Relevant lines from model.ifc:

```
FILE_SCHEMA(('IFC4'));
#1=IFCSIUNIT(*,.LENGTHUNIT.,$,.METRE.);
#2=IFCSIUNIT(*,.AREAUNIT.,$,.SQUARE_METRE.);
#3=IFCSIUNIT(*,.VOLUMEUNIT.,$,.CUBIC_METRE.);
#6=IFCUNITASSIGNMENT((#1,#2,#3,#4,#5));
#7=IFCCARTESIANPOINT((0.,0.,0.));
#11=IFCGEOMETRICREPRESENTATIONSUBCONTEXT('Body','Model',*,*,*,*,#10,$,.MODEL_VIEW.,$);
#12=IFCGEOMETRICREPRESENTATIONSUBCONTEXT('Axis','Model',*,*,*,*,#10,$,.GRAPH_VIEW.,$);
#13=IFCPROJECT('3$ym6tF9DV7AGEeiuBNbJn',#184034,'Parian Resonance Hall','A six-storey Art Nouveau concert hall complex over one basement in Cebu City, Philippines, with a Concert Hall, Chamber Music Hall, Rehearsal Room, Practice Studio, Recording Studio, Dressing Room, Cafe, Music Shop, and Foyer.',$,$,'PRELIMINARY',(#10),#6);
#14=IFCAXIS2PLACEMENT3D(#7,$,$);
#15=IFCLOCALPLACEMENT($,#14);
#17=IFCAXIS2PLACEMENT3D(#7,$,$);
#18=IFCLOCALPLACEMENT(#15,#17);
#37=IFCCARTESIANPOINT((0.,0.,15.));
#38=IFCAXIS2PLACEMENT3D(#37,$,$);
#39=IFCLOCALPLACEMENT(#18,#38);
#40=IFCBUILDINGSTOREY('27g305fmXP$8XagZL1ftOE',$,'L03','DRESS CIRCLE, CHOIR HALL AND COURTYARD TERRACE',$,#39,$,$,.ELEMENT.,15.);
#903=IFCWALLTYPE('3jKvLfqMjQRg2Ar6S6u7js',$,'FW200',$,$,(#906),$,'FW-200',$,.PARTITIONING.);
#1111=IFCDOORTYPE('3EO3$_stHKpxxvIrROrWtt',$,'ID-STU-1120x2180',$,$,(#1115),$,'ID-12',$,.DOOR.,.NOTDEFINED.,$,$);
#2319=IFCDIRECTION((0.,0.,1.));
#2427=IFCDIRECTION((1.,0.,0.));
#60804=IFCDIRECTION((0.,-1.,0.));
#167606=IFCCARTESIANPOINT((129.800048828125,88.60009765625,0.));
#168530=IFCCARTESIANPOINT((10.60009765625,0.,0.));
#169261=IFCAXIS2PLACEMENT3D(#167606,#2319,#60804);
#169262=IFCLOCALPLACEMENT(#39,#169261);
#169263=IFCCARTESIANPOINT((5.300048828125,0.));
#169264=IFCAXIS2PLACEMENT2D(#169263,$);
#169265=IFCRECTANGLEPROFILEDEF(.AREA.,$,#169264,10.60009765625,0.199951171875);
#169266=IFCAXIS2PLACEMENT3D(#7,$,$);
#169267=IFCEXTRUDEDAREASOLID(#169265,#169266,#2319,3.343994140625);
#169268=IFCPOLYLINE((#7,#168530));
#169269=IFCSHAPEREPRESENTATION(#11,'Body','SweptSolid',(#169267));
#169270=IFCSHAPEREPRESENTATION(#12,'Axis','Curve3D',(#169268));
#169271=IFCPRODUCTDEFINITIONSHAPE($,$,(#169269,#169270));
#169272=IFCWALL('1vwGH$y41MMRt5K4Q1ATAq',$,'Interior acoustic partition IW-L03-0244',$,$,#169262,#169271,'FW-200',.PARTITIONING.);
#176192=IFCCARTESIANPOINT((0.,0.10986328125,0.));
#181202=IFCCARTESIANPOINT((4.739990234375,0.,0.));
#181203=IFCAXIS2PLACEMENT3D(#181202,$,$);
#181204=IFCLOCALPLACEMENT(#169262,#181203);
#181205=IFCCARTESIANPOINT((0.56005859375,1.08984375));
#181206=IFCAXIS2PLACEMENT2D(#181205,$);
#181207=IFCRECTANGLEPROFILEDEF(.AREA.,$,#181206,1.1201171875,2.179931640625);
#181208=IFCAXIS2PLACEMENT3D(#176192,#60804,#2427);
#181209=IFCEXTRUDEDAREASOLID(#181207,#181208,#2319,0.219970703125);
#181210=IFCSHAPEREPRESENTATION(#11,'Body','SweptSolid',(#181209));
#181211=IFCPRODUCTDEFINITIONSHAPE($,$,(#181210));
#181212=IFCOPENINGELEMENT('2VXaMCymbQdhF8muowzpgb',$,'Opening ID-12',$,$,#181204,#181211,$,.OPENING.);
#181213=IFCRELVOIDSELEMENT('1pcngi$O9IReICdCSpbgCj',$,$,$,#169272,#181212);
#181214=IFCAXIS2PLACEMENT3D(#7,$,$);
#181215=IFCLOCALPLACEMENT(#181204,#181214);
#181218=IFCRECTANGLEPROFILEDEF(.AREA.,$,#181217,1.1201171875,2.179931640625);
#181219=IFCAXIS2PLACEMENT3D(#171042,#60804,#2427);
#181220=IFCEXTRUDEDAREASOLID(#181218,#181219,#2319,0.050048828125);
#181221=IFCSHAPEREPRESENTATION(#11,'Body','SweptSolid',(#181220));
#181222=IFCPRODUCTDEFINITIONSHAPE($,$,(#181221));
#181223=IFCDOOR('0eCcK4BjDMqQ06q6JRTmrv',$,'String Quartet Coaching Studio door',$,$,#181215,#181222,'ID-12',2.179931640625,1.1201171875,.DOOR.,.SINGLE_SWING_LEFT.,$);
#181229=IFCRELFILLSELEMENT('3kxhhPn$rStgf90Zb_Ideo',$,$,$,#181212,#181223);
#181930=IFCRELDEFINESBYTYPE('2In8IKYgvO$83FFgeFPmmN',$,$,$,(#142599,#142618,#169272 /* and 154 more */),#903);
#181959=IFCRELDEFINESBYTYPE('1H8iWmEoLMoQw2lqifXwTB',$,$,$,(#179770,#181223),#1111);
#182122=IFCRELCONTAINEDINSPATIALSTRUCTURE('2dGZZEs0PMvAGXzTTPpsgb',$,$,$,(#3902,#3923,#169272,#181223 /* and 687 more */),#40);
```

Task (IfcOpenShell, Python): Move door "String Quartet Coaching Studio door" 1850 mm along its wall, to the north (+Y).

```python
import ifcopenshell
import ifcopenshell.api.geometry
import ifcopenshell.util.placement
import ifcopenshell.util.unit

model = ifcopenshell.open("model.ifc")
unit_scale = ifcopenshell.util.unit.calculate_unit_scale(model)

door = model.by_guid("0eCcK4BjDMqQ06q6JRTmrv")
opening = door.FillsVoids[0].RelatingOpeningElement
wall = opening.VoidsElements[0].RelatingBuildingElement

wall_matrix = ifcopenshell.util.placement.get_local_placement(wall.ObjectPlacement)
shift = wall_matrix[:3, 0] * -1.85 / unit_scale
before = ifcopenshell.util.placement.get_local_placement(door.ObjectPlacement)[:3, 3].copy()

# The door is placed relative to its opening, so it follows when the opening moves.
matrix = ifcopenshell.util.placement.get_local_placement(opening.ObjectPlacement)
matrix[:3, 3] += shift
ifcopenshell.api.geometry.edit_object_placement(
    model, product=opening, matrix=matrix, is_si=False, should_transform_children=True
)

after = ifcopenshell.util.placement.get_local_placement(door.ObjectPlacement)[:3, 3]
print("door moved by", (after - before).round(3) + 0.0)

model.write("model_updated.ifc")
```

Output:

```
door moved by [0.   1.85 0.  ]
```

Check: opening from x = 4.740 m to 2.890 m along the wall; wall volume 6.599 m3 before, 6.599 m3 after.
